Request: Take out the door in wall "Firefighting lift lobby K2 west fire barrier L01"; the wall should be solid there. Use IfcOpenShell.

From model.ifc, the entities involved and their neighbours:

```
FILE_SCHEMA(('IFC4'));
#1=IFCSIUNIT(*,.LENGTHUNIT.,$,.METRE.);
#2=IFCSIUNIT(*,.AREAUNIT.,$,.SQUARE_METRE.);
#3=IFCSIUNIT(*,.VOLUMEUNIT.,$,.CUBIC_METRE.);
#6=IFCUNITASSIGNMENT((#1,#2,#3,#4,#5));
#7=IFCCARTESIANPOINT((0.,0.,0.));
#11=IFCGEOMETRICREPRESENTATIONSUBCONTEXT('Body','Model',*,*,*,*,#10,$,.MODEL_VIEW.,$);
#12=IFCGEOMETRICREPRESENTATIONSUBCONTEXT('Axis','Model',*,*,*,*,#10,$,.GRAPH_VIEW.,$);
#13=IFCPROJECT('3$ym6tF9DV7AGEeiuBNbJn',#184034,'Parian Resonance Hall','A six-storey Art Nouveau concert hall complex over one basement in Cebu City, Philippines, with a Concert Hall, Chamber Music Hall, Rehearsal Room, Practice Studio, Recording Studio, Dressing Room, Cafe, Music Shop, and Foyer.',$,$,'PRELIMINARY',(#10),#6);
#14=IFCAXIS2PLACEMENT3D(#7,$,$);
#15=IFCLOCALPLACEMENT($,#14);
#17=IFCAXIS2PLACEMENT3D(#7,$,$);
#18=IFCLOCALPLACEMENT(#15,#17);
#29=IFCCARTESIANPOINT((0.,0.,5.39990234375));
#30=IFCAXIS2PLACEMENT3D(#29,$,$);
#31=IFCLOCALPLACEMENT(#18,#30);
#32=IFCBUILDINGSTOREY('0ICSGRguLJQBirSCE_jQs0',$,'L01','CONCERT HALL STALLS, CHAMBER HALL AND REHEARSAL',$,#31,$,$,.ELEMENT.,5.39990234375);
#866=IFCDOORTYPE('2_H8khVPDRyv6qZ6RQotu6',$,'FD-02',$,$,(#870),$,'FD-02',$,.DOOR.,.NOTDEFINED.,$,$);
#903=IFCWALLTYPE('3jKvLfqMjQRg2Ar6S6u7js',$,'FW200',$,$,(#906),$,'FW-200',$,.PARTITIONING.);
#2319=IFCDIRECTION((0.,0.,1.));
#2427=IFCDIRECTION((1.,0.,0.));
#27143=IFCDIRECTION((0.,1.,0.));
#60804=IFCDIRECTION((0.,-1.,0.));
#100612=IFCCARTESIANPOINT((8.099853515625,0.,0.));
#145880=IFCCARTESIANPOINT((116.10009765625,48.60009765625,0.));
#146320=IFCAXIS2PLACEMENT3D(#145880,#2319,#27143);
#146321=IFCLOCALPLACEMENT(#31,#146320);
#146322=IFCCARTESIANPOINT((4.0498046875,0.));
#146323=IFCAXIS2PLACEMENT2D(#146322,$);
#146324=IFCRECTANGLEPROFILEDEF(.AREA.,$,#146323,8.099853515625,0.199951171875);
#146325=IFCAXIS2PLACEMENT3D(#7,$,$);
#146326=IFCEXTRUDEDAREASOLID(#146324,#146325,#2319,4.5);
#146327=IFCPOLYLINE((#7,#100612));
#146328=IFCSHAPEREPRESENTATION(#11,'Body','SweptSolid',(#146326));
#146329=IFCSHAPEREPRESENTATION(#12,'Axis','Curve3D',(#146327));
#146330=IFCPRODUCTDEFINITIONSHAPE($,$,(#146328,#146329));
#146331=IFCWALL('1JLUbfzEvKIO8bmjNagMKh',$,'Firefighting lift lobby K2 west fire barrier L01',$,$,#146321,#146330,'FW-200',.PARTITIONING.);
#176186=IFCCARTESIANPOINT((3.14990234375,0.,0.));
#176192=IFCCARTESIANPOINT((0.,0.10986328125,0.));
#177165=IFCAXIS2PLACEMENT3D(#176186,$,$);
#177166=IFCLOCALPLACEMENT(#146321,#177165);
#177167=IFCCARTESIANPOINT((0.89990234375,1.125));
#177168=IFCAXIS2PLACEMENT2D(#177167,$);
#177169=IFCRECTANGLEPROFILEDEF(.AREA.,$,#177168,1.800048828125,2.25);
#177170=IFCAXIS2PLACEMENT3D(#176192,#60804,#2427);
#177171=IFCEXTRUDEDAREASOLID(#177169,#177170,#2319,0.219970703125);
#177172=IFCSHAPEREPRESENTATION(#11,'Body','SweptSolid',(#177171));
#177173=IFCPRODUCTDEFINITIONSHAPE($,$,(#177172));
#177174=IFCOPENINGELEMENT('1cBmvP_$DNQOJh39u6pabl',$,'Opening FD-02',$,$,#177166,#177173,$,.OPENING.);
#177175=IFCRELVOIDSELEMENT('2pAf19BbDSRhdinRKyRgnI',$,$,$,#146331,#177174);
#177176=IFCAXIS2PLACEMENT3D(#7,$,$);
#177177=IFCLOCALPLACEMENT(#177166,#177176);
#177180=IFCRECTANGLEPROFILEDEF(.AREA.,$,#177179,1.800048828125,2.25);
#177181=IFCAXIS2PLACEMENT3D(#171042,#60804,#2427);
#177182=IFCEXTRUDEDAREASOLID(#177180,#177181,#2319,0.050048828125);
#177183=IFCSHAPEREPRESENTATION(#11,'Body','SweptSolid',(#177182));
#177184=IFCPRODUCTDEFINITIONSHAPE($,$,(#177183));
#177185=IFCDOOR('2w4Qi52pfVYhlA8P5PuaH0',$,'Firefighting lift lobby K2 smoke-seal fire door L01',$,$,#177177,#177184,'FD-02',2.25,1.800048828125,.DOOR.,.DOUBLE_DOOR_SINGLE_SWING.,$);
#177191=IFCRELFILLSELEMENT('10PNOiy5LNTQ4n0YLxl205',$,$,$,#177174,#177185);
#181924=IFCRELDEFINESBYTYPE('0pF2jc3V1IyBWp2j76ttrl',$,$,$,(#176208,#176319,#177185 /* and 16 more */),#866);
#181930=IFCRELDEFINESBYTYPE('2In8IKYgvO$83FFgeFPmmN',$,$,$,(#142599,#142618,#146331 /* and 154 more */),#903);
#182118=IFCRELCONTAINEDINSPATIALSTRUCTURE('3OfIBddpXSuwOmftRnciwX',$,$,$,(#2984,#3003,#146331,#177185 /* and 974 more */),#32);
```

```python
import ifcopenshell
import ifcopenshell.api.feature
import ifcopenshell.api.root
import ifcopenshell.geom
import ifcopenshell.util.shape

model = ifcopenshell.open("model.ifc")
settings = ifcopenshell.geom.settings()


def volume(element):
    """Net volume in cubic metres, openings subtracted."""
    shape = ifcopenshell.geom.create_shape(settings, element)
    return ifcopenshell.util.shape.get_volume(shape.geometry)


door = model.by_guid("2w4Qi52pfVYhlA8P5PuaH0")
opening = door.FillsVoids[0].RelatingOpeningElement
wall = opening.VoidsElements[0].RelatingBuildingElement
before = volume(wall)

ifcopenshell.api.root.remove_product(model, product=door)
ifcopenshell.api.feature.remove_feature(model, feature=opening)

after = volume(wall)

print(f"wall volume {before:.3f} -> {after:.3f} m3")

model.write("model_updated.ifc")
```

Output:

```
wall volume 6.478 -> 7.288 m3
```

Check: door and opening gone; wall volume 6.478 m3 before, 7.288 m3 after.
